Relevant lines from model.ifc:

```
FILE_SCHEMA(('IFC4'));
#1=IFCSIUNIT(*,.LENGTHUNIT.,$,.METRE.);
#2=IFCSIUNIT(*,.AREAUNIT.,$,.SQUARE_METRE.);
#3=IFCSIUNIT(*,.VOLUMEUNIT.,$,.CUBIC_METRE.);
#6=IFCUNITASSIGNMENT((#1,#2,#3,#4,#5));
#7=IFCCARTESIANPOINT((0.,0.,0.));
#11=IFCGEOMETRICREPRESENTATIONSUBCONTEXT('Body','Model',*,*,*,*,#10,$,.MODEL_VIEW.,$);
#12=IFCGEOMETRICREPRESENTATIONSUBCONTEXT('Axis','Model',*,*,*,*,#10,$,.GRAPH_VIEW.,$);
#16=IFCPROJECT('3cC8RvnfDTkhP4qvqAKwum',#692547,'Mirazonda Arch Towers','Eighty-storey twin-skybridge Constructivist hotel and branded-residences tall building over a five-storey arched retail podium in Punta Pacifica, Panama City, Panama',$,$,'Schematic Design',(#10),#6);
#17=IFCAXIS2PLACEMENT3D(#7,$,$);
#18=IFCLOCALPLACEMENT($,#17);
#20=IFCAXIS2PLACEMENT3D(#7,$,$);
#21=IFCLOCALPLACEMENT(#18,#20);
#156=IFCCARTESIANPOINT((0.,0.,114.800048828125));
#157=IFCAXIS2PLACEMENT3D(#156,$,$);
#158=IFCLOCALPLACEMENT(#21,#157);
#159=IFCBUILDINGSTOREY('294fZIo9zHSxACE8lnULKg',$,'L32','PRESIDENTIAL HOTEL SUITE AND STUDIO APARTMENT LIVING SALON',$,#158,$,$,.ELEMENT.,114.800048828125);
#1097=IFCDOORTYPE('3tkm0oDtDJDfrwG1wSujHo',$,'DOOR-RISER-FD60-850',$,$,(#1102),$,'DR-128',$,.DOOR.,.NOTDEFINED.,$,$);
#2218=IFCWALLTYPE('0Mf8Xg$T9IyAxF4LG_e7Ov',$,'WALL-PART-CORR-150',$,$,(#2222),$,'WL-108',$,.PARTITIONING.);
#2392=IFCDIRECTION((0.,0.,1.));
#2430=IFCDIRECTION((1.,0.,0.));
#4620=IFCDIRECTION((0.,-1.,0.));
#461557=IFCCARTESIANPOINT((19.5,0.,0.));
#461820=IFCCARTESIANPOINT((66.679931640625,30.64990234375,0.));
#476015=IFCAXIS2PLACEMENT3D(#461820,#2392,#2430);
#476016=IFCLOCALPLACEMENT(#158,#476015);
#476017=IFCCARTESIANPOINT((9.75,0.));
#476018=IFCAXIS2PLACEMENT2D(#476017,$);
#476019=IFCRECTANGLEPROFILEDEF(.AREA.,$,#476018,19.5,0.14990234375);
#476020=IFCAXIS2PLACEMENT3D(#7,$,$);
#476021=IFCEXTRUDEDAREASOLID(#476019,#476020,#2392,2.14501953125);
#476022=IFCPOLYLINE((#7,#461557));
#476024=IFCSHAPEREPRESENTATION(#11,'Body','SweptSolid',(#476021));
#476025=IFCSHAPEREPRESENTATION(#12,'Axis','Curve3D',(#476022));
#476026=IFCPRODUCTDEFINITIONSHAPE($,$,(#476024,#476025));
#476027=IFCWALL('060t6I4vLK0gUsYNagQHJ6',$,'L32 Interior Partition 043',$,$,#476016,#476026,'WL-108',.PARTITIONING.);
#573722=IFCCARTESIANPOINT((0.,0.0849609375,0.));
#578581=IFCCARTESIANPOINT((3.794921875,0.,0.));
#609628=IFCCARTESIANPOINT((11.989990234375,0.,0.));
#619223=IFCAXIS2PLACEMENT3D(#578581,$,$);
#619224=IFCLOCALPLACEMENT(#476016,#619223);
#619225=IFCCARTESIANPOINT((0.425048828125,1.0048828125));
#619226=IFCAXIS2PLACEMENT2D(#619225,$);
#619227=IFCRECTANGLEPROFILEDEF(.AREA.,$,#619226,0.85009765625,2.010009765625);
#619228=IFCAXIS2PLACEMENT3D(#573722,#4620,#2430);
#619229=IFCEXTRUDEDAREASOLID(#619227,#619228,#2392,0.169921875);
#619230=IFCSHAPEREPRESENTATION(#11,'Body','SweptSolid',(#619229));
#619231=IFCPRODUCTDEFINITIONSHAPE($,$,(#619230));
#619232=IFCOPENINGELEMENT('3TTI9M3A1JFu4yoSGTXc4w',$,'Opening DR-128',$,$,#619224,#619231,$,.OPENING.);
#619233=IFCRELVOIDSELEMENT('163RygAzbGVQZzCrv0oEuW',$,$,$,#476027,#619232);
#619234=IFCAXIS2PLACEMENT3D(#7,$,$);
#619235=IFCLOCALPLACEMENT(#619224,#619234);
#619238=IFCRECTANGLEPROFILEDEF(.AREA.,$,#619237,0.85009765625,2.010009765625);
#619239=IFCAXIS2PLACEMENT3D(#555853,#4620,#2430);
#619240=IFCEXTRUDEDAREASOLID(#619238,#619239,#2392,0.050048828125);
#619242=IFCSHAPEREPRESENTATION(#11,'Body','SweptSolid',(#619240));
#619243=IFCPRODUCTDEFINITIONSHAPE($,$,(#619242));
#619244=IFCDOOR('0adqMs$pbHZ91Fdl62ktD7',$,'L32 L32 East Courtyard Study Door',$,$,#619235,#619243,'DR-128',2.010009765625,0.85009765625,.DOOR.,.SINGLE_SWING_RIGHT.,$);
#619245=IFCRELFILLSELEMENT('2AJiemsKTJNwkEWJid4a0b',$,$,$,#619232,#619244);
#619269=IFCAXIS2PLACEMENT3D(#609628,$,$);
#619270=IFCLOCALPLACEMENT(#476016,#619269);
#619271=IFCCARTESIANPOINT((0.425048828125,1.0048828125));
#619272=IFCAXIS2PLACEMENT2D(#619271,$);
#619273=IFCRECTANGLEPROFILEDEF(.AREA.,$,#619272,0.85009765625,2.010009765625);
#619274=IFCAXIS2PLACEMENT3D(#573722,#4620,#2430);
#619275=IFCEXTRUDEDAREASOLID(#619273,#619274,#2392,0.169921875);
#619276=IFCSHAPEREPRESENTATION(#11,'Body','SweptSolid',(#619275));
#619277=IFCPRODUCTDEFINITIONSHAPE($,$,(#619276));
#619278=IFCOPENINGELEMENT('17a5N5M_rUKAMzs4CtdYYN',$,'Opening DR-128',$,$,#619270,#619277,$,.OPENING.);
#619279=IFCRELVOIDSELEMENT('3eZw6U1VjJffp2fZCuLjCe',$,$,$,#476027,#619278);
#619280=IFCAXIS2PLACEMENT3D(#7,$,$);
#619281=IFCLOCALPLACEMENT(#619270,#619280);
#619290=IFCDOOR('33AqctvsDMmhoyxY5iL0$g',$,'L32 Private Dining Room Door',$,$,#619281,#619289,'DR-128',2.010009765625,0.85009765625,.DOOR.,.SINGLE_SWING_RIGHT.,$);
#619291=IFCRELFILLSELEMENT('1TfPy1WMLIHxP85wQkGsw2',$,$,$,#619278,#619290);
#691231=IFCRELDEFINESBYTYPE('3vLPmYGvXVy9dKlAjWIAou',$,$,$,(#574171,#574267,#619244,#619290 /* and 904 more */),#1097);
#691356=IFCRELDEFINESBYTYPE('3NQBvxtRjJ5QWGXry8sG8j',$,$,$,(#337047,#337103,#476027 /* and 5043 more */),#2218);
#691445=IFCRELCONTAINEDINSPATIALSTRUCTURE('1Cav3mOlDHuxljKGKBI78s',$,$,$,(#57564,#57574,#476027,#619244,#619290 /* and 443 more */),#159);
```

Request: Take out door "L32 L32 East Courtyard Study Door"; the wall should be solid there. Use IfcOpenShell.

```python
import ifcopenshell
import ifcopenshell.api.feature
import ifcopenshell.api.root
import ifcopenshell.geom
import ifcopenshell.util.shape

model = ifcopenshell.open("model.ifc")
settings = ifcopenshell.geom.settings()


def volume(element):
    """Net volume in cubic metres, openings subtracted."""
    shape = ifcopenshell.geom.create_shape(settings, element)
    return ifcopenshell.util.shape.get_volume(shape.geometry)


door = model.by_guid("0adqMs$pbHZ91Fdl62ktD7")
opening = door.FillsVoids[0].RelatingOpeningElement
wall = opening.VoidsElements[0].RelatingBuildingElement
before = volume(wall)

ifcopenshell.api.root.remove_product(model, product=door)
ifcopenshell.api.feature.remove_feature(model, feature=opening)

after = volume(wall)

print(f"wall volume {before:.3f} -> {after:.3f} m3")

model.write("model-out.ifc")
```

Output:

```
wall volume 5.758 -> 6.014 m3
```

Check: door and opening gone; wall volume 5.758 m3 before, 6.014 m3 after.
